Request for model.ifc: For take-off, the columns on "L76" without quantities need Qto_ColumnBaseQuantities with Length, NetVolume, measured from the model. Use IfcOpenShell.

First a look at what the model holds.

```python
import ifcopenshell
import ifcopenshell.util.element
import ifcopenshell.util.unit

model = ifcopenshell.open("model.ifc")
print(model.schema)
for unit_type in ("LENGTHUNIT", "AREAUNIT", "VOLUMEUNIT"):
    print(unit_type, ifcopenshell.util.unit.calculate_unit_scale(model, unit_type))
storey = next(s for s in model.by_type("IfcBuildingStorey") if s.Name == "L76")
columns = [e for e in ifcopenshell.util.element.get_decomposition(storey) if e.is_a("IfcColumn")]
for e in sorted(columns, key=lambda e: e.id()):
    print(e.id(), e.is_a(), e.Name, list(ifcopenshell.util.element.get_psets(e, qtos_only=True)), sep=" | ")
```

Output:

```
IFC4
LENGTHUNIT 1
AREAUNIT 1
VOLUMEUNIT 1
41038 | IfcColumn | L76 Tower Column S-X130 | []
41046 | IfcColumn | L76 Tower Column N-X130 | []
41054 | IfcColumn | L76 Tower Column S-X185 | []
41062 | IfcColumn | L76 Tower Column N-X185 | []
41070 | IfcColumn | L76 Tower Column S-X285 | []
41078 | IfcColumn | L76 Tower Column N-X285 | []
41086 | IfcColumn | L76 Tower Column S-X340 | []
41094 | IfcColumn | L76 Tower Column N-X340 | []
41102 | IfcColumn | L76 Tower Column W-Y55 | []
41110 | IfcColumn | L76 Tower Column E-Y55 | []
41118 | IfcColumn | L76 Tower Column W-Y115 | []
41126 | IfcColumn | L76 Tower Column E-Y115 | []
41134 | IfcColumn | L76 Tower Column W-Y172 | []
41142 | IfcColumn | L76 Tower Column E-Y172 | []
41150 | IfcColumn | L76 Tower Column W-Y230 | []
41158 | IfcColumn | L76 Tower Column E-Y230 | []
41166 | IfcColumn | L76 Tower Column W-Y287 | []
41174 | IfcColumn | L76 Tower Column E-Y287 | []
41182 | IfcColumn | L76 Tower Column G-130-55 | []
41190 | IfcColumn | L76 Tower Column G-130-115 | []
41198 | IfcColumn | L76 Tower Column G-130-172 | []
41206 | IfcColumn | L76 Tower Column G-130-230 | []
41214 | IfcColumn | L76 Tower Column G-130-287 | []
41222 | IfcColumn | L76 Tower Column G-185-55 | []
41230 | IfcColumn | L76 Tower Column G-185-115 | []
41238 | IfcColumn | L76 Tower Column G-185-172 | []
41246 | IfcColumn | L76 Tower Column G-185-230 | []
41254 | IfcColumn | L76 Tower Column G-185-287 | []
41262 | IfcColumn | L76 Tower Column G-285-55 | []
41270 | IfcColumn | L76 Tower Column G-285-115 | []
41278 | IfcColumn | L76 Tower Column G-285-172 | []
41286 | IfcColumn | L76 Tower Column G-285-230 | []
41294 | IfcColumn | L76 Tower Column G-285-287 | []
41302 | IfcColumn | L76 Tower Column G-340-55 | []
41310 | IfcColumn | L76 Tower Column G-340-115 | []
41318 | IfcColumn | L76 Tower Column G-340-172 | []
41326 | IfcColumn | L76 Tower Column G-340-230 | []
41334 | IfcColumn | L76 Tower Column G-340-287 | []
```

```python
import ifcopenshell
import ifcopenshell.api.pset
import ifcopenshell.geom
import ifcopenshell.util.element
import ifcopenshell.util.shape
import ifcopenshell.util.unit

model = ifcopenshell.open("model.ifc")
unit_scale = ifcopenshell.util.unit.calculate_unit_scale(model)
volume_scale = ifcopenshell.util.unit.calculate_unit_scale(model, "VOLUMEUNIT")
settings = ifcopenshell.geom.settings()

storey = next(s for s in model.by_type("IfcBuildingStorey") if s.Name == "L76")
columns = [e for e in ifcopenshell.util.element.get_decomposition(storey) if e.is_a("IfcColumn")]

for e in sorted(columns, key=lambda e: e.id()):
    if ifcopenshell.util.element.get_psets(e, qtos_only=True, should_inherit=False):
        continue
    # Geometry comes back in metres, in the element's own axes.
    shape = ifcopenshell.geom.create_shape(settings, e)
    values = {
        "Length": ifcopenshell.util.shape.get_z(shape.geometry) / unit_scale,
        "NetVolume": ifcopenshell.util.shape.get_volume(shape.geometry) / volume_scale,
    }
    qto = ifcopenshell.api.pset.add_qto(model, product=e, name="Qto_ColumnBaseQuantities")
    ifcopenshell.api.pset.edit_qto(model, qto=qto, properties=values)
    print(e.id(), {k: round(v, 3) for k, v in values.items()})

model.write("model_v2.ifc")
```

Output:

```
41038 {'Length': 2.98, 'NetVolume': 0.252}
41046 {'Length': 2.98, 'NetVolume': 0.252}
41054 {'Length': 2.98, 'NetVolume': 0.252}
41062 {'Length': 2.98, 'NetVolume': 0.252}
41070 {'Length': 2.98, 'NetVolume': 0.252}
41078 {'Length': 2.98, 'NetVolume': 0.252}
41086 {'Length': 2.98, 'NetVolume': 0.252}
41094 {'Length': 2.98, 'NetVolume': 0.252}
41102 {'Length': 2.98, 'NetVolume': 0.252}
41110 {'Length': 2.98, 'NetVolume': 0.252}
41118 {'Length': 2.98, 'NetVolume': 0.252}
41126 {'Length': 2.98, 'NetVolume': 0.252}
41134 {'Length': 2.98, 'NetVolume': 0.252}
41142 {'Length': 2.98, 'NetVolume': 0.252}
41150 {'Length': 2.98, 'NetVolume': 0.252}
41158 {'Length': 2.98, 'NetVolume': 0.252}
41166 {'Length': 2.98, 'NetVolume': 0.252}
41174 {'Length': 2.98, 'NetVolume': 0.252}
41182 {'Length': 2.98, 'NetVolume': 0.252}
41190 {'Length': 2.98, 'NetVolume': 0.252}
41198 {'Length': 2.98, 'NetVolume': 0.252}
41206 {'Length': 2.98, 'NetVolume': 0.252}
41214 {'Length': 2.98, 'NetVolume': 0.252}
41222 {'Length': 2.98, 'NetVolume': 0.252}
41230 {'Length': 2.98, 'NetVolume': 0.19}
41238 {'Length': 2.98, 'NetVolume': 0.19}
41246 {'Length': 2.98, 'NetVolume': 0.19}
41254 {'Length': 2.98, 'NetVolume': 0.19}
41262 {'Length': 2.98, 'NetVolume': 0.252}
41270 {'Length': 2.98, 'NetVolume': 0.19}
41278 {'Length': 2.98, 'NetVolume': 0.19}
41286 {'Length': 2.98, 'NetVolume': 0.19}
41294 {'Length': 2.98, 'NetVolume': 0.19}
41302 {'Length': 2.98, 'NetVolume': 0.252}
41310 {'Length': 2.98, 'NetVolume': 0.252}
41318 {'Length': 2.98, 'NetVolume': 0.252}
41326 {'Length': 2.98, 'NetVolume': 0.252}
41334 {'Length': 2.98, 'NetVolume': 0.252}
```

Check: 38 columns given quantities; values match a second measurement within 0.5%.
